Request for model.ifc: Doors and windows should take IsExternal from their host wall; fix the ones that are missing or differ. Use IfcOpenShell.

First a look at what the model holds.

```python
import ifcopenshell
import ifcopenshell.util.element

model = ifcopenshell.open("model.ifc")
print(model.schema)
seen = {}
for e in model.by_type("IfcDoor") + model.by_type("IfcWindow"):
    if not e.FillsVoids:
        continue
    host = e.FillsVoids[0].RelatingOpeningElement.VoidsElements[0].RelatingBuildingElement
    own = ifcopenshell.util.element.get_pset(e, f"Pset_{e.is_a()[3:].removesuffix('StandardCase')}Common", "IsExternal")
    wall = ifcopenshell.util.element.get_pset(host, "Pset_WallCommon", "IsExternal")
    seen[e.is_a(), own, wall] = seen.get((e.is_a(), own, wall), 0) + 1
for (cls, own, wall), count in sorted(seen.items(), key=str):
    print(count, cls, "IsExternal:", own, "| host wall:", wall)
```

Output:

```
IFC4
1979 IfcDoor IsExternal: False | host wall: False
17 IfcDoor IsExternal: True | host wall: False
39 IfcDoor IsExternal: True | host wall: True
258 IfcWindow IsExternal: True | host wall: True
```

```python
import ifcopenshell
import ifcopenshell.api.pset
import ifcopenshell.util.element

model = ifcopenshell.open("model.ifc")

count = 0
for ifc_class, pset_name in (("IfcDoor", "Pset_DoorCommon"), ("IfcWindow", "Pset_WindowCommon")):
    for e in model.by_type(ifc_class):
        if not e.FillsVoids:
            continue
        host = e.FillsVoids[0].RelatingOpeningElement.VoidsElements[0].RelatingBuildingElement
        external = ifcopenshell.util.element.get_pset(host, "Pset_WallCommon", "IsExternal")
        if external is None or ifcopenshell.util.element.get_pset(e, pset_name, "IsExternal") == external:
            continue
        pset = ifcopenshell.api.pset.add_pset(model, product=e, name=pset_name)
        ifcopenshell.api.pset.edit_pset(model, pset=pset, properties={"IsExternal": external})
        count += 1

print(count, "updated")

model.write("model_v2.ifc")
```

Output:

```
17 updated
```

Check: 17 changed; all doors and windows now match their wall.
